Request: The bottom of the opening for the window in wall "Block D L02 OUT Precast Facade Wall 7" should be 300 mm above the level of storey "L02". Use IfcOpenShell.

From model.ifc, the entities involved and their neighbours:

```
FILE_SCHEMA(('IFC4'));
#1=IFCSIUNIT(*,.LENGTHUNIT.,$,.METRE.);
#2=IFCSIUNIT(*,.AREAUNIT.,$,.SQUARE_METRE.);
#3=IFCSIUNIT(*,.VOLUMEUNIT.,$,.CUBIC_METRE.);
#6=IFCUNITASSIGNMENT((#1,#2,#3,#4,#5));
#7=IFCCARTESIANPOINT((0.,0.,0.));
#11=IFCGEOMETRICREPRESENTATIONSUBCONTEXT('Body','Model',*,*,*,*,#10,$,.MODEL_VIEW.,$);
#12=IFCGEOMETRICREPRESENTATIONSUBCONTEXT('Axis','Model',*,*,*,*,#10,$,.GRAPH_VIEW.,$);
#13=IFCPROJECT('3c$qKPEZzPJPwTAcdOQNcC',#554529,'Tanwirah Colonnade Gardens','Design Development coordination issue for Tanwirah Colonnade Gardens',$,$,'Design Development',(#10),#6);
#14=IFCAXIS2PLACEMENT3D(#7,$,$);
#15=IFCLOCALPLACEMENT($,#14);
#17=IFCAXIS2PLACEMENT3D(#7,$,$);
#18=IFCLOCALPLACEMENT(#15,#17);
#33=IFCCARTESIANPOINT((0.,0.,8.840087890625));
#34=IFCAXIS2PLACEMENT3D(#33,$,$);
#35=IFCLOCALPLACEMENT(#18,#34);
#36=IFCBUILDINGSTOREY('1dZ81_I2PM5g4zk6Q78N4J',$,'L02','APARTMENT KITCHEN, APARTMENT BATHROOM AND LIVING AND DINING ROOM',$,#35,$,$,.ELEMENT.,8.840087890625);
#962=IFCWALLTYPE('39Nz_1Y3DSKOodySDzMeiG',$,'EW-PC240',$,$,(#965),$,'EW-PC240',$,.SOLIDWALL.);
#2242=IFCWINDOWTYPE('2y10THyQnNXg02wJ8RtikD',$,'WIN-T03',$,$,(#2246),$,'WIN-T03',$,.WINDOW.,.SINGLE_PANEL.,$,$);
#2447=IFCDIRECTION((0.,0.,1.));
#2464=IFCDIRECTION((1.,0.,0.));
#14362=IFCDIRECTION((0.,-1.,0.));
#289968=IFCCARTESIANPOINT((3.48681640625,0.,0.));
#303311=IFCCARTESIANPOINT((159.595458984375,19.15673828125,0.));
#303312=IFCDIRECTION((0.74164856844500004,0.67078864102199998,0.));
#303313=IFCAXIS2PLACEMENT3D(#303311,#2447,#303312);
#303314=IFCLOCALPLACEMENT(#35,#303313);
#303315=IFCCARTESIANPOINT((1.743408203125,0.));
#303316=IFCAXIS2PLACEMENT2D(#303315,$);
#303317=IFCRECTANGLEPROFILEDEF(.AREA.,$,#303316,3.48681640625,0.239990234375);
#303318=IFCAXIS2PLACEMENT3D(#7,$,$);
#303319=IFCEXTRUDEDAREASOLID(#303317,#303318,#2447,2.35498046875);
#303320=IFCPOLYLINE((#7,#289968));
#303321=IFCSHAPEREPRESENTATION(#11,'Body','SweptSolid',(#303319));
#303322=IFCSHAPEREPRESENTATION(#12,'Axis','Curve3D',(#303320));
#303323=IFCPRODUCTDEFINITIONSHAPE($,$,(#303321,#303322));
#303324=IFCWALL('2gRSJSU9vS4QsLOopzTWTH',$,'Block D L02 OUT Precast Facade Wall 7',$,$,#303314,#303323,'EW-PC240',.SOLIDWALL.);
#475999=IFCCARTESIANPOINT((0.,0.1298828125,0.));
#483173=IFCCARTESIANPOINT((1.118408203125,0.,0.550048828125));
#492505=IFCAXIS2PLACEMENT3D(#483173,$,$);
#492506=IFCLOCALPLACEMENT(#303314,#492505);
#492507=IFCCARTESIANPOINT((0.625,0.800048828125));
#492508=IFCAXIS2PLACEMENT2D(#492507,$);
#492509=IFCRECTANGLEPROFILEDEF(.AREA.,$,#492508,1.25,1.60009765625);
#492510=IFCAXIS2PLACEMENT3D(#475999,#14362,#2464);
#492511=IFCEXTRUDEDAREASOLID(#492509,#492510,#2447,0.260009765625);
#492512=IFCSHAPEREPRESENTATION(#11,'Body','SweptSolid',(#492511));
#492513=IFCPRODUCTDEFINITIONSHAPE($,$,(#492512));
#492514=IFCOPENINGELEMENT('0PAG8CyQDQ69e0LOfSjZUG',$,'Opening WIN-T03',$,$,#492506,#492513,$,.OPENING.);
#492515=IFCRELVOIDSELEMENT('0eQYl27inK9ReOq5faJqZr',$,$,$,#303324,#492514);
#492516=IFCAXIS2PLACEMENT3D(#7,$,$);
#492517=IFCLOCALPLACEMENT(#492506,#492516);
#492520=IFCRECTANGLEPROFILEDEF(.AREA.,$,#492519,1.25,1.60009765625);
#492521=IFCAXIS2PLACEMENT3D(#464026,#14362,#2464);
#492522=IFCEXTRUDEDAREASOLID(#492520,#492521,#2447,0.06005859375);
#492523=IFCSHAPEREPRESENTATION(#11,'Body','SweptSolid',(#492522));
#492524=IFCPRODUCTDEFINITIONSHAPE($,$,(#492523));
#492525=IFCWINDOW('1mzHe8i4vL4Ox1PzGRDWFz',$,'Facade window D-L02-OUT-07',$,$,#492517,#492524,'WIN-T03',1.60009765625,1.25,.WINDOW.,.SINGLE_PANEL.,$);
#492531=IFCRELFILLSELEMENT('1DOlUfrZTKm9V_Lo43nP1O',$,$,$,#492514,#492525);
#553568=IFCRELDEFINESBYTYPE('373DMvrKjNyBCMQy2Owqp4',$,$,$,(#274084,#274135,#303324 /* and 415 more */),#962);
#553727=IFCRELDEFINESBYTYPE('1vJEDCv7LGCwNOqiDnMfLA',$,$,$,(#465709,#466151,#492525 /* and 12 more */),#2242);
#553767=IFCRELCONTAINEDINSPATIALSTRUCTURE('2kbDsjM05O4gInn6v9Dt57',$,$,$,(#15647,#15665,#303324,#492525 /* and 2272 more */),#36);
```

```python
import numpy as np
import ifcopenshell
import ifcopenshell.api.geometry
import ifcopenshell.geom
import ifcopenshell.util.element
import ifcopenshell.util.placement
import ifcopenshell.util.shape
import ifcopenshell.util.unit

model = ifcopenshell.open("model.ifc")
unit_scale = ifcopenshell.util.unit.calculate_unit_scale(model)

window = model.by_id(492525)
opening = window.FillsVoids[0].RelatingOpeningElement
storey = ifcopenshell.util.element.get_container(window, ifc_class="IfcBuildingStorey")
level = ifcopenshell.util.placement.get_local_placement(storey.ObjectPlacement)[2, 3]

# The opening's origin need not be at the sill, so measure its lowest point.
shape = ifcopenshell.geom.create_shape(ifcopenshell.geom.settings(), opening)
bottom = ifcopenshell.util.shape.get_shape_bottom_elevation(shape, shape.geometry) / unit_scale
dz = level + 0.3 / unit_scale - bottom

shift = np.array([0.0, 0.0, dz])
# The window is placed relative to its opening, so it follows when the opening moves.
matrix = ifcopenshell.util.placement.get_local_placement(opening.ObjectPlacement)
matrix[:3, 3] += shift
ifcopenshell.api.geometry.edit_object_placement(
    model, product=opening, matrix=matrix, is_si=False, should_transform_children=True
)

print(f"moved by {dz * unit_scale:+.3f} m")

model.write("model_v2.ifc")
```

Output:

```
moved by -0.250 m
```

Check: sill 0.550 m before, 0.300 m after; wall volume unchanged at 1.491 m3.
